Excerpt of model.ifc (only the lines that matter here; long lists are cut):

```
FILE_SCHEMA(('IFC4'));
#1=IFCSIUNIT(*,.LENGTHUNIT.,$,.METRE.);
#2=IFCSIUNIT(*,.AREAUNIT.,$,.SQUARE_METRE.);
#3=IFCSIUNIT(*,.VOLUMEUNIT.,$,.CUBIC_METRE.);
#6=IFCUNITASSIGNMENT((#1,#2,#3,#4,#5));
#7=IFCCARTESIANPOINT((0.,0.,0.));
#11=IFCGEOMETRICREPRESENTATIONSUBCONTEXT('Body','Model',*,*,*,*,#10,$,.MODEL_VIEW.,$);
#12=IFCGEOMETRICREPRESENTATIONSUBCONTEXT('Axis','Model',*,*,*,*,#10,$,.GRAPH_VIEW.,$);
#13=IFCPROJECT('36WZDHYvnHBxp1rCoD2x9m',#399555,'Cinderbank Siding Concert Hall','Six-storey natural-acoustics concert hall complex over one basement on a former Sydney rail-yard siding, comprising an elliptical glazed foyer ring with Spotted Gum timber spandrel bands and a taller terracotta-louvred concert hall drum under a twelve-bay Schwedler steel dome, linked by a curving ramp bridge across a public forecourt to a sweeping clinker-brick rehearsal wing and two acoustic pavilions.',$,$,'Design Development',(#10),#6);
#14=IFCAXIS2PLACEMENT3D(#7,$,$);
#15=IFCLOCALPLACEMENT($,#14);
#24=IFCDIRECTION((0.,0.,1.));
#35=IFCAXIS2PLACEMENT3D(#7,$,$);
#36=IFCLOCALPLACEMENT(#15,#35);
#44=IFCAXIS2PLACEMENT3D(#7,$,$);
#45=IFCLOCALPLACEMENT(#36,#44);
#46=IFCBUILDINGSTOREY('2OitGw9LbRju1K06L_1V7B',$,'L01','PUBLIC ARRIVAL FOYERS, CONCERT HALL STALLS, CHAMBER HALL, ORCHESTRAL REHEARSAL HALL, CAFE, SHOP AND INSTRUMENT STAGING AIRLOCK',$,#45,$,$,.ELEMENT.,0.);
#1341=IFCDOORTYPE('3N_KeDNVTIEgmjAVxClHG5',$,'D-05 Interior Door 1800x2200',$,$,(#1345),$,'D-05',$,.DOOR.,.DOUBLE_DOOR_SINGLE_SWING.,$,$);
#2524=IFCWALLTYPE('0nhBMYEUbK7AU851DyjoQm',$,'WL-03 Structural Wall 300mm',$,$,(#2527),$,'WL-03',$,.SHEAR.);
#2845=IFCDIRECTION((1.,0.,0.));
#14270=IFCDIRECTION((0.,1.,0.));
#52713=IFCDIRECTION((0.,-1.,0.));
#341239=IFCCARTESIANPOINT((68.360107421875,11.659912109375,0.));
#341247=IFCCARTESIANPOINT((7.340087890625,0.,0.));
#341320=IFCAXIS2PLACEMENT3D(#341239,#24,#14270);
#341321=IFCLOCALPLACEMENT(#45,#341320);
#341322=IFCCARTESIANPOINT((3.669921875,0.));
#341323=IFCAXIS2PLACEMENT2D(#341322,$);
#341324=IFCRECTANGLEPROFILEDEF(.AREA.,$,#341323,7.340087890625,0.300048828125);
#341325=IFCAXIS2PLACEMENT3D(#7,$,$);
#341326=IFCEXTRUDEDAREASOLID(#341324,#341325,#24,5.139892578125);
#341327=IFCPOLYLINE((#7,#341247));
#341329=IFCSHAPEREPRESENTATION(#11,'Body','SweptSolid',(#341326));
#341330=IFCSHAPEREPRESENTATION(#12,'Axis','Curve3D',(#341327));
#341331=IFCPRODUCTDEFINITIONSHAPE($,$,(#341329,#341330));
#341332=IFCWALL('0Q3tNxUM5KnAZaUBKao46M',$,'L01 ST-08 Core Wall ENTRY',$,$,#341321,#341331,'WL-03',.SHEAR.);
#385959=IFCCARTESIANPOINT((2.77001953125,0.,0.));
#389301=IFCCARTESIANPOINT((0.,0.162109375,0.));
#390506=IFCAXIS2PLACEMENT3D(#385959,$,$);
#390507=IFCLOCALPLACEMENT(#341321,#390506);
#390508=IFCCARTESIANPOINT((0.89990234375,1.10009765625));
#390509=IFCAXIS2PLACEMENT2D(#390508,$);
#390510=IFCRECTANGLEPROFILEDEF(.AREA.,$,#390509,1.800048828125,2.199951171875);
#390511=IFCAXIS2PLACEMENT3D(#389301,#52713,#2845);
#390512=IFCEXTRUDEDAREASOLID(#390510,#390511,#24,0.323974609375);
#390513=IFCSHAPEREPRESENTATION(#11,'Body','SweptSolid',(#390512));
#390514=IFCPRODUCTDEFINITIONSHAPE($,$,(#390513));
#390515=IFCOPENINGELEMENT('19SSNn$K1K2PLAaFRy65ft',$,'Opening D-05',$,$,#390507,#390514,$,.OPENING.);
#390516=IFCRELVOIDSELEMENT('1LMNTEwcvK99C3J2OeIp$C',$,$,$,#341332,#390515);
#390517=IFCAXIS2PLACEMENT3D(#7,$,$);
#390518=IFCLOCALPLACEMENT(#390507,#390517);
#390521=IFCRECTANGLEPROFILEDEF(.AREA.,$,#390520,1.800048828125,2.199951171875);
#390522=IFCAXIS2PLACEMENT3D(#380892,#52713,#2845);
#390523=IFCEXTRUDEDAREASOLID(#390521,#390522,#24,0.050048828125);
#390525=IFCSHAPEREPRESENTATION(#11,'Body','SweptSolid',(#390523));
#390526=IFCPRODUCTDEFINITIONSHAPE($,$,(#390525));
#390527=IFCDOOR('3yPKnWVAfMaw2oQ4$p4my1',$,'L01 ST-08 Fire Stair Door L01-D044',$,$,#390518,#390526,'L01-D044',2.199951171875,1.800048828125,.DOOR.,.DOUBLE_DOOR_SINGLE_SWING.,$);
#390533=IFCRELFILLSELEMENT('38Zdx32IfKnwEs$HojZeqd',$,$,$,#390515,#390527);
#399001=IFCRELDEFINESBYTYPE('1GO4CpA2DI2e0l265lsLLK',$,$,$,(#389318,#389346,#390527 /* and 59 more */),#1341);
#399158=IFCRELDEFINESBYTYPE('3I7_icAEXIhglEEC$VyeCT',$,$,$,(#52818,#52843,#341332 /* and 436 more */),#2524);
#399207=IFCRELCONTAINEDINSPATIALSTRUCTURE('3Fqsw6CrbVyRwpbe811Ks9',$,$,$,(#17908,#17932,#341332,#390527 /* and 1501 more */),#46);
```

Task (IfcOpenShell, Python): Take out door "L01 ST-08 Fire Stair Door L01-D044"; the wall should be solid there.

```python
import ifcopenshell
import ifcopenshell.api.feature
import ifcopenshell.api.root
import ifcopenshell.geom
import ifcopenshell.util.shape

model = ifcopenshell.open("model.ifc")
settings = ifcopenshell.geom.settings()


def volume(element):
    """Net volume in cubic metres, openings subtracted."""
    shape = ifcopenshell.geom.create_shape(settings, element)
    return ifcopenshell.util.shape.get_volume(shape.geometry)


door = model.by_guid("3yPKnWVAfMaw2oQ4$p4my1")
opening = door.FillsVoids[0].RelatingOpeningElement
wall = opening.VoidsElements[0].RelatingBuildingElement
before = volume(wall)

ifcopenshell.api.root.remove_product(model, product=door)
ifcopenshell.api.feature.remove_feature(model, feature=opening)

after = volume(wall)

print(f"wall volume {before:.3f} -> {after:.3f} m3")

model.write("model_v2.ifc")
```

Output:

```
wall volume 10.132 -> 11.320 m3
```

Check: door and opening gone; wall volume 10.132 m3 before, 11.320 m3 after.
